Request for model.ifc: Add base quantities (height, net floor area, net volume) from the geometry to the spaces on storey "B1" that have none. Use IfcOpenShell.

First a look at what the model holds.

```python
import ifcopenshell
import ifcopenshell.util.element
import ifcopenshell.util.unit

model = ifcopenshell.open("model.ifc")
print(model.schema)
for unit_type in ("LENGTHUNIT", "AREAUNIT", "VOLUMEUNIT"):
    print(unit_type, ifcopenshell.util.unit.calculate_unit_scale(model, unit_type))
storey = next(s for s in model.by_type("IfcBuildingStorey") if s.Name == "B1")
spaces = [e for e in ifcopenshell.util.element.get_decomposition(storey) if e.is_a("IfcSpace")]
for e in sorted(spaces, key=lambda e: e.id()):
    print(e.id(), e.is_a(), e.Name, list(ifcopenshell.util.element.get_psets(e, qtos_only=True)), sep=" | ")
```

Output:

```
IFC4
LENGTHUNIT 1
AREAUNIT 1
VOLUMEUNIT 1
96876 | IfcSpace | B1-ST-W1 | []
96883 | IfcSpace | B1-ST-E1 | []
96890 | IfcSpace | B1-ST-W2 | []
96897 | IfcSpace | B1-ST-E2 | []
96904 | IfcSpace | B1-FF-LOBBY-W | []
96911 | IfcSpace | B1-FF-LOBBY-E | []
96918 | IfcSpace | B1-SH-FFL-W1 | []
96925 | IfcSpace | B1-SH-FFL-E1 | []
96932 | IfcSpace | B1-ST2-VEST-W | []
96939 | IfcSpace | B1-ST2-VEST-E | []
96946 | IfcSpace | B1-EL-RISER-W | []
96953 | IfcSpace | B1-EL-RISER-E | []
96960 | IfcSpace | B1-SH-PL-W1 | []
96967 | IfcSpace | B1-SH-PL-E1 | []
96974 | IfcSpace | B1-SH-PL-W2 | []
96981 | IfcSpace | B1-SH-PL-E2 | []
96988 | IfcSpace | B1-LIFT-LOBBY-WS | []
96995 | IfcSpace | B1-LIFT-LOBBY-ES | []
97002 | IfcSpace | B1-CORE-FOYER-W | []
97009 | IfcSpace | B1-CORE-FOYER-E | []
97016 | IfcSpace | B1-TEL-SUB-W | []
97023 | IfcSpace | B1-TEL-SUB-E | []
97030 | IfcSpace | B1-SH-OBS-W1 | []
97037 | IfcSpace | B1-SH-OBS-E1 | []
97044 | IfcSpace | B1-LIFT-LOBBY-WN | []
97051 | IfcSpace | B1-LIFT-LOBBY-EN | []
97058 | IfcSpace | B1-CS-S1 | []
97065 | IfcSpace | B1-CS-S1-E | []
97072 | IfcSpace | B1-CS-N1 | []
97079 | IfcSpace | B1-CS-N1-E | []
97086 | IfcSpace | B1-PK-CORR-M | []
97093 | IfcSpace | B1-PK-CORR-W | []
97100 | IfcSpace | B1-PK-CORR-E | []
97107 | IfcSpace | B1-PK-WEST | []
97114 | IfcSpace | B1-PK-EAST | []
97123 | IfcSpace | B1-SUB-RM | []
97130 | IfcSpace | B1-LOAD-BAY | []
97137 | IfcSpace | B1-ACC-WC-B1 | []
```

```python
import ifcopenshell
import ifcopenshell.api.pset
import ifcopenshell.geom
import ifcopenshell.util.element
import ifcopenshell.util.shape
import ifcopenshell.util.unit

model = ifcopenshell.open("model.ifc")
unit_scale = ifcopenshell.util.unit.calculate_unit_scale(model)
area_scale = ifcopenshell.util.unit.calculate_unit_scale(model, "AREAUNIT")
volume_scale = ifcopenshell.util.unit.calculate_unit_scale(model, "VOLUMEUNIT")
settings = ifcopenshell.geom.settings()

storey = next(s for s in model.by_type("IfcBuildingStorey") if s.Name == "B1")
spaces = [e for e in ifcopenshell.util.element.get_decomposition(storey) if e.is_a("IfcSpace")]

for e in sorted(spaces, key=lambda e: e.id()):
    if ifcopenshell.util.element.get_psets(e, qtos_only=True, should_inherit=False):
        continue
    # Geometry comes back in metres, in the element's own axes.
    shape = ifcopenshell.geom.create_shape(settings, e)
    values = {
        "Height": ifcopenshell.util.shape.get_z(shape.geometry) / unit_scale,
        "NetFloorArea": ifcopenshell.util.shape.get_footprint_area(shape.geometry) / area_scale,
        "NetVolume": ifcopenshell.util.shape.get_volume(shape.geometry) / volume_scale,
    }
    qto = ifcopenshell.api.pset.add_qto(model, product=e, name="Qto_SpaceBaseQuantities")
    ifcopenshell.api.pset.edit_qto(model, qto=qto, properties=values)
    print(e.id(), {k: round(v, 3) for k, v in values.items()})

model.write("model_rev.ifc")
```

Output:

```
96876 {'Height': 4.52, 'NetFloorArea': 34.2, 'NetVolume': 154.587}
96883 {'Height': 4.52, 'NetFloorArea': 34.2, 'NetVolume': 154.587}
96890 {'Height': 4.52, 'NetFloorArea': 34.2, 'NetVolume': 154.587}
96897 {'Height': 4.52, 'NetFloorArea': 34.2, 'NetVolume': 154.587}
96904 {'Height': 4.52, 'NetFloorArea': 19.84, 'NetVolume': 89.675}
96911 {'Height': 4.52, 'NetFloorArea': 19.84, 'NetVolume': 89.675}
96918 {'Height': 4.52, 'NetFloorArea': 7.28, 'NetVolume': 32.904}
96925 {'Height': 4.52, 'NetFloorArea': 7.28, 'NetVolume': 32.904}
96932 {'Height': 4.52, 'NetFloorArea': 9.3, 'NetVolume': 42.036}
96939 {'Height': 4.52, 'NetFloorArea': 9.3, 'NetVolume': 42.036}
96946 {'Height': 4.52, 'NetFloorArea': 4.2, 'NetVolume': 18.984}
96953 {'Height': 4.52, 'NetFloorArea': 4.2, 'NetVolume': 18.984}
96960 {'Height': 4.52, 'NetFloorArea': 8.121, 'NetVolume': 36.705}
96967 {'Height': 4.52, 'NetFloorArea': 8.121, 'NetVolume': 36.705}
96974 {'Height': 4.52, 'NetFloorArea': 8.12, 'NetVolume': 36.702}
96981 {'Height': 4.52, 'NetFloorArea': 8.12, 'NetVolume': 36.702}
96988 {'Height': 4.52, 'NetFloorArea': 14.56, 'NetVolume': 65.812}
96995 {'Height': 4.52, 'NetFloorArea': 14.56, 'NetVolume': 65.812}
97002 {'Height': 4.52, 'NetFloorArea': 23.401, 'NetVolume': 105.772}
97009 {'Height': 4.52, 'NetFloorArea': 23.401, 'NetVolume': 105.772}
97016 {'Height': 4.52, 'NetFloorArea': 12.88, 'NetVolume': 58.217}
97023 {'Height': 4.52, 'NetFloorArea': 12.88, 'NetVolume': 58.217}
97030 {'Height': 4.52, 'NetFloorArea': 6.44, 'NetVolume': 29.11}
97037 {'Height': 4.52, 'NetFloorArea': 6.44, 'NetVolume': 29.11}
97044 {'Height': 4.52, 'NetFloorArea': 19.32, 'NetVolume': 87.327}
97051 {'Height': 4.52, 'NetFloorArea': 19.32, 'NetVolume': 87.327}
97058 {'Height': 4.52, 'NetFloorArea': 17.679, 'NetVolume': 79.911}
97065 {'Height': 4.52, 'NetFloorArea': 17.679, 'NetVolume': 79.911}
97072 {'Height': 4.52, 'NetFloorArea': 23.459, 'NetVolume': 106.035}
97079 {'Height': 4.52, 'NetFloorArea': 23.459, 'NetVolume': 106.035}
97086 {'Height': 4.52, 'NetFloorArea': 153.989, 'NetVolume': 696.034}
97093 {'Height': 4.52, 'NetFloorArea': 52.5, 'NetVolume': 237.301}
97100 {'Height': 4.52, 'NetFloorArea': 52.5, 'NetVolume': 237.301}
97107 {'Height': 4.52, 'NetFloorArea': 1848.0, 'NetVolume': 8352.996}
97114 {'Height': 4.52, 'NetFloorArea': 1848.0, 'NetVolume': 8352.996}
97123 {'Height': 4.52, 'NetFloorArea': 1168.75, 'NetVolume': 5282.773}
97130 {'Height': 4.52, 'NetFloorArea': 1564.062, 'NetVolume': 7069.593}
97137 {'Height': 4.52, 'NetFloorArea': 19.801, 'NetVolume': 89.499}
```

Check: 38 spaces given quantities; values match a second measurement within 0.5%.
